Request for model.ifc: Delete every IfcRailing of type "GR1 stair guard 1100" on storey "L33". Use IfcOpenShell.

First a look at what the model holds.

```python
import ifcopenshell
import ifcopenshell.util.element

model = ifcopenshell.open("model.ifc")
print(model.schema)
storey = next(s for s in model.by_type("IfcBuildingStorey") if s.Name == "L33")
railings = [e for e in ifcopenshell.util.element.get_decomposition(storey) if e.is_a("IfcRailing")]
seen = {}
for e in railings:
    element_type = ifcopenshell.util.element.get_type(e)
    name = element_type.Name if element_type not in (None, e) else None
    seen[name] = seen.get(name, 0) + 1
for name, count in sorted(seen.items(), key=str):
    print(count, "x", name)
```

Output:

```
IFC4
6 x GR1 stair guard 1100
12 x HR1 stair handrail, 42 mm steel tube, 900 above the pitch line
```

```python
import ifcopenshell
import ifcopenshell.api.root
import ifcopenshell.util.element

model = ifcopenshell.open("model.ifc")

storey = next(s for s in model.by_type("IfcBuildingStorey") if s.Name == "L33")
railings = [e for e in ifcopenshell.util.element.get_decomposition(storey) if e.is_a("IfcRailing")]
targets = [e for e in railings if (t := ifcopenshell.util.element.get_type(e)) not in (None, e) and t.Name == "GR1 stair guard 1100"]

for e in targets:
    ifcopenshell.api.root.remove_product(model, product=e)
print(len(targets), "removed")

model.write("model_edited.ifc")
```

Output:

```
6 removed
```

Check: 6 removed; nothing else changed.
